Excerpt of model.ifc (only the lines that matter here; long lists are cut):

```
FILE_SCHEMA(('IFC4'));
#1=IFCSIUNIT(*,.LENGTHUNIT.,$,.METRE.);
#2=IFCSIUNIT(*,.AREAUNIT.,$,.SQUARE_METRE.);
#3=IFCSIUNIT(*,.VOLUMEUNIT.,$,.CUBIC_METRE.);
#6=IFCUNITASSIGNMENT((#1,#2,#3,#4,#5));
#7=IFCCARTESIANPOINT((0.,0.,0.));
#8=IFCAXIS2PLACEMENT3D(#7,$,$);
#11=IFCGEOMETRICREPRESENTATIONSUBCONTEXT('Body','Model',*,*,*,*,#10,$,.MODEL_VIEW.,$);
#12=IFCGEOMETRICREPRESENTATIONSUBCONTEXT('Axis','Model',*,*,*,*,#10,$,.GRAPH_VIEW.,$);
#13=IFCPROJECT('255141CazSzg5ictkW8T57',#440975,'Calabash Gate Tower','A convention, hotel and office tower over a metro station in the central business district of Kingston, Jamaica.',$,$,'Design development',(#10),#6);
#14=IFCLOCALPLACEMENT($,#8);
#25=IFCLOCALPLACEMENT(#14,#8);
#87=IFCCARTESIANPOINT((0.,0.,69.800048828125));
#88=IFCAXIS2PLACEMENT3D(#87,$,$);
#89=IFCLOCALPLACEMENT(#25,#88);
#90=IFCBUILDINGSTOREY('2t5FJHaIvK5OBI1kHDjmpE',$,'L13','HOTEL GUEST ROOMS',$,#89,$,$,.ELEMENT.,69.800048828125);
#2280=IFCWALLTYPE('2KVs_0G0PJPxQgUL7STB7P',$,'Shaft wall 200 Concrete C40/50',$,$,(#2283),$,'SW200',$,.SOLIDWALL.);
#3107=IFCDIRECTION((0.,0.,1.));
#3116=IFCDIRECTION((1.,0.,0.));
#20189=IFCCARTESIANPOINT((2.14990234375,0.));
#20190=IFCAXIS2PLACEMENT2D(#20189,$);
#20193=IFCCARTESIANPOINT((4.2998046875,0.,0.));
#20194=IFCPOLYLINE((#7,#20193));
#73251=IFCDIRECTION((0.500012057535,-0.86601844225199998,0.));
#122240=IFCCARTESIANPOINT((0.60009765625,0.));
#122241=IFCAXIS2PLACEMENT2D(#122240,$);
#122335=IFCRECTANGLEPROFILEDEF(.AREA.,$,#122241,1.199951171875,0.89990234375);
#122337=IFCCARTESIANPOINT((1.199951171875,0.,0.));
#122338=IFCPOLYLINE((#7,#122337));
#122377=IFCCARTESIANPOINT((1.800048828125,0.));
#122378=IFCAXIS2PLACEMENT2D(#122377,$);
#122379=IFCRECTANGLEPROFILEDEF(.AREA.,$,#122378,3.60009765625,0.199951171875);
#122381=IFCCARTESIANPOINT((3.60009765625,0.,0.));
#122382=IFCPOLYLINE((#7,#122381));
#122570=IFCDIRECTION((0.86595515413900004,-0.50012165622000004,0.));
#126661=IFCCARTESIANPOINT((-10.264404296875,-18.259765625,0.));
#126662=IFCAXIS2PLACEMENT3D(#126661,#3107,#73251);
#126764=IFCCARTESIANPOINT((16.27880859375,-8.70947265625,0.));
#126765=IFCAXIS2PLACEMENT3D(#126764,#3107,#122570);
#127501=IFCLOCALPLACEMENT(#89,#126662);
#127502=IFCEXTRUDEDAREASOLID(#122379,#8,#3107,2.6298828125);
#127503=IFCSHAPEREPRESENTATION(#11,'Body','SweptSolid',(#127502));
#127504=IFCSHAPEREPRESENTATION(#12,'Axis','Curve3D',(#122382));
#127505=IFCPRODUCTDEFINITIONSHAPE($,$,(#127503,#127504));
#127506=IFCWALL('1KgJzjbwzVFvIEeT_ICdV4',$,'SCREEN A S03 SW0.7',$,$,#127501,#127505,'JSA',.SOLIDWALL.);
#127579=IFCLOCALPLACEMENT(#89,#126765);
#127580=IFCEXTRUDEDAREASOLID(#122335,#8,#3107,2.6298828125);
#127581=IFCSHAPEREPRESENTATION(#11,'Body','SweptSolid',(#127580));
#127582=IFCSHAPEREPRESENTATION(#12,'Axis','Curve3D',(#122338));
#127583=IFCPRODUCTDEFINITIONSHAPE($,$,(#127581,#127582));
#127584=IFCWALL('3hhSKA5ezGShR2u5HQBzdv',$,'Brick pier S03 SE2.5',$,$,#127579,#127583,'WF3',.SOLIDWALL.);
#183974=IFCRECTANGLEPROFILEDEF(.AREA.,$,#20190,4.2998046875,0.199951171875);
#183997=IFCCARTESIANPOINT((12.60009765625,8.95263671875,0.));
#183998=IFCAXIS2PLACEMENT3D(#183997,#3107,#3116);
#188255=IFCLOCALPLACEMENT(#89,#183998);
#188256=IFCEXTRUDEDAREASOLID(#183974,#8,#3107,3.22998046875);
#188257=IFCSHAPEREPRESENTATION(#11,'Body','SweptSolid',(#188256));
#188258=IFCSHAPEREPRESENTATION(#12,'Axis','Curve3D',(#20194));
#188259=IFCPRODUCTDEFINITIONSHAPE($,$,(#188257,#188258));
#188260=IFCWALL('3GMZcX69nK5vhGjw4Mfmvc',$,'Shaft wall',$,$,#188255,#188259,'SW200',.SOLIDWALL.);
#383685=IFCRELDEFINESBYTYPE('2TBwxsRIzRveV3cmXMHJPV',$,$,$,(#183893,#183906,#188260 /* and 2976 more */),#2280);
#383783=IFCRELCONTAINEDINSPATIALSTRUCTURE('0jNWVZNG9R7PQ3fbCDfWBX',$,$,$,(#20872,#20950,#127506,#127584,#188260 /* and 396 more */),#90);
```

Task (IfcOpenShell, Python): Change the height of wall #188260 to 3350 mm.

```python
import ifcopenshell
import ifcopenshell.geom
import ifcopenshell.util.representation
import ifcopenshell.util.shape
import ifcopenshell.util.unit

model = ifcopenshell.open("model.ifc")
unit_scale = ifcopenshell.util.unit.calculate_unit_scale(model)
settings = ifcopenshell.geom.settings()


def volume(element):
    """Net volume in cubic metres, openings subtracted."""
    shape = ifcopenshell.geom.create_shape(settings, element)
    return ifcopenshell.util.shape.get_volume(shape.geometry)


wall = model.by_guid("3GMZcX69nK5vhGjw4Mfmvc")
before = volume(wall)

body = ifcopenshell.util.representation.get_representation(wall, "Model", "Body")
solid = body.Items[0]
old_height = solid.Depth
solid.Depth = 3.35 / unit_scale
after = volume(wall)

print(f"height {old_height:g} -> {solid.Depth:g}, volume {before:.3f} -> {after:.3f} m3")

model.write("model-out.ifc")
```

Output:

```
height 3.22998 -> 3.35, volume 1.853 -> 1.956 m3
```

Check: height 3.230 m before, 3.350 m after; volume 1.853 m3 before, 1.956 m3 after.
